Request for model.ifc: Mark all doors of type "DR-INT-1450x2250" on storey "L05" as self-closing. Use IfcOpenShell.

First a look at what the model holds.

```python
import ifcopenshell
import ifcopenshell.util.element

model = ifcopenshell.open("model.ifc")
print(model.schema)
storey = next(s for s in model.by_type("IfcBuildingStorey") if s.Name == "L05")
doors = [e for e in ifcopenshell.util.element.get_decomposition(storey) if e.is_a("IfcDoor")]
seen = {}
for e in doors:
    element_type = ifcopenshell.util.element.get_type(e)
    key = (element_type.Name if element_type != e and element_type else None, ifcopenshell.util.element.get_pset(e, "Pset_DoorCommon", "SelfClosing"))
    seen[key] = seen.get(key, 0) + 1
for (name, value), count in sorted(seen.items(), key=str):
    print(count, "x", name, "|", value)
```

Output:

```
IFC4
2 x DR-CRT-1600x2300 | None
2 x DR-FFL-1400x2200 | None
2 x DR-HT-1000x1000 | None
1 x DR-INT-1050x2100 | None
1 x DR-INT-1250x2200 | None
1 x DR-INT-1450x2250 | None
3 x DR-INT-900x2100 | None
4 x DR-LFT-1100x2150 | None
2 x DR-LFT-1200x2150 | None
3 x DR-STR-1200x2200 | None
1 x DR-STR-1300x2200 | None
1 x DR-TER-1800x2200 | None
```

```python
import ifcopenshell
import ifcopenshell.api.pset
import ifcopenshell.util.element

model = ifcopenshell.open("model.ifc")

storey = next(s for s in model.by_type("IfcBuildingStorey") if s.Name == "L05")
doors = [e for e in ifcopenshell.util.element.get_decomposition(storey) if e.is_a("IfcDoor")]

count = 0
for e in doors:
    element_type = ifcopenshell.util.element.get_type(e)
    if element_type in (None, e) or element_type.Name != "DR-INT-1450x2250":
        continue
    # add_pset returns the element's existing set when there is one.
    pset = ifcopenshell.api.pset.add_pset(model, product=e, name="Pset_DoorCommon")
    ifcopenshell.api.pset.edit_pset(model, pset=pset, properties={"SelfClosing": True})
    count += 1

print(count, "doors updated")

model.write("model-out.ifc")
```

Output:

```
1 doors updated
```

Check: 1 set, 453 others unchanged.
